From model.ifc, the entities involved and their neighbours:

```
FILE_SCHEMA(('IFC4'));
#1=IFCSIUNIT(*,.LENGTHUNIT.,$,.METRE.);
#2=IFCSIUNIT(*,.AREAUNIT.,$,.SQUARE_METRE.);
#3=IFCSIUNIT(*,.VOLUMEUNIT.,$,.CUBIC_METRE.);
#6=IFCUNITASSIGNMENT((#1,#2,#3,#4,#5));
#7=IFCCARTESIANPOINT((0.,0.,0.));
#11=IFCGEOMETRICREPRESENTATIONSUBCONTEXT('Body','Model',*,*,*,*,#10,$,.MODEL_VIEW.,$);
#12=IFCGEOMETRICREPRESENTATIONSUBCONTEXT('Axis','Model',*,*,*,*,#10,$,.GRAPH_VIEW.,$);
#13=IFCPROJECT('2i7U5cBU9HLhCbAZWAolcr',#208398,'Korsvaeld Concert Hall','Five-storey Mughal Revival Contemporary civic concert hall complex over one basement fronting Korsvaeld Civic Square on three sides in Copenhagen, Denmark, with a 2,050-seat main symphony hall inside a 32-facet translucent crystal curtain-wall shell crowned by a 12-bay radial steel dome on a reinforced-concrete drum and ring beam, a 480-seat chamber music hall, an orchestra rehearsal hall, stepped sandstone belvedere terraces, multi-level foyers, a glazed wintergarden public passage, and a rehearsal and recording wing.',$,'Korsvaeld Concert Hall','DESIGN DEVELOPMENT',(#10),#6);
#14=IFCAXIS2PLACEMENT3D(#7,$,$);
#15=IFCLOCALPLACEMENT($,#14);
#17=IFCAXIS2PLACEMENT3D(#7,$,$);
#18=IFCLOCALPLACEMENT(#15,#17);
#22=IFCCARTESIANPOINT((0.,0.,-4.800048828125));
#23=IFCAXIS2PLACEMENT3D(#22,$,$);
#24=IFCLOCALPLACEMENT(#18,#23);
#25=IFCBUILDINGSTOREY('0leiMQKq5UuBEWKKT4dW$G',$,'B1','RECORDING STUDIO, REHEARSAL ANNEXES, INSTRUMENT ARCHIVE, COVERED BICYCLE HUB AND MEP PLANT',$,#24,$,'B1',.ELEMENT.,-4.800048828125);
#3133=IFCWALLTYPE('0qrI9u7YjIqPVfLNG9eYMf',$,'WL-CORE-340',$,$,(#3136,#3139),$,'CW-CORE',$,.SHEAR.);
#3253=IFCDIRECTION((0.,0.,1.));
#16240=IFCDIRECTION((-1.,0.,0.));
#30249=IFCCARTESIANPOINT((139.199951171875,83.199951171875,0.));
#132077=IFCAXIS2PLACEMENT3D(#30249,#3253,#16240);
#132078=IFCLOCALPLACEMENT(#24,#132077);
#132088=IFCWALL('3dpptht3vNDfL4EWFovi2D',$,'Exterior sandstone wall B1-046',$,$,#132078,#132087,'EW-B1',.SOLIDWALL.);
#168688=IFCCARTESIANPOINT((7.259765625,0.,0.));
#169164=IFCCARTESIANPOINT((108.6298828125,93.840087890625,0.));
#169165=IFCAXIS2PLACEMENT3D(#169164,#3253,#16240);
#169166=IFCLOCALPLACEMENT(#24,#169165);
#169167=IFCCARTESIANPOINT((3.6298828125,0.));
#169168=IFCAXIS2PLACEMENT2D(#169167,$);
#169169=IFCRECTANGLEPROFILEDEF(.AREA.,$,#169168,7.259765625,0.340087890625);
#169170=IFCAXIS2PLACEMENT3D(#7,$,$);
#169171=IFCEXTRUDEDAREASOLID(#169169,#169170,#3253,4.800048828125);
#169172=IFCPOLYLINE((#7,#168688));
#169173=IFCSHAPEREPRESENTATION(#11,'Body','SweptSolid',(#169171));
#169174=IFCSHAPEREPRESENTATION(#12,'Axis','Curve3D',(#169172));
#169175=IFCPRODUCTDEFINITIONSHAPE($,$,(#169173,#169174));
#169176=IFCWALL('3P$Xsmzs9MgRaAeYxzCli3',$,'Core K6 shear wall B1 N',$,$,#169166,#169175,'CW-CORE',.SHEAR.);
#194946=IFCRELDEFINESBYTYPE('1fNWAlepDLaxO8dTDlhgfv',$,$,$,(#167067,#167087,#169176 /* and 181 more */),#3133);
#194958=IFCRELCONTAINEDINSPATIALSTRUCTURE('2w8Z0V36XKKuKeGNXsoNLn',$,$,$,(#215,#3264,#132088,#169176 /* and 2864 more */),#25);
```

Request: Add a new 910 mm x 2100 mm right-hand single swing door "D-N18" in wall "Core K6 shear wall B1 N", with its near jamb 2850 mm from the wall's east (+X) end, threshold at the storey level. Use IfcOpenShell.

```python
import numpy as np
import ifcopenshell
import ifcopenshell.api.feature
import ifcopenshell.api.geometry
import ifcopenshell.api.root
import ifcopenshell.api.spatial
import ifcopenshell.geom
import ifcopenshell.util.element
import ifcopenshell.util.placement
import ifcopenshell.util.representation
import ifcopenshell.util.shape
import ifcopenshell.util.unit

model = ifcopenshell.open("model.ifc")
unit_scale = ifcopenshell.util.unit.calculate_unit_scale(model)
settings = ifcopenshell.geom.settings()


def volume(element):
    """Net volume in cubic metres, openings subtracted."""
    shape = ifcopenshell.geom.create_shape(settings, element)
    return ifcopenshell.util.shape.get_volume(shape.geometry)


wall = model.by_guid("3P$Xsmzs9MgRaAeYxzCli3")
storey = ifcopenshell.util.element.get_container(wall, ifc_class="IfcBuildingStorey")
context = ifcopenshell.util.representation.get_context(model, "Model", "Body", "MODEL_VIEW")
before = volume(wall)

width, height, from_end, sill = 0.91, 2.1, 2.85, 0.0  # metres

# The wall runs along its own X axis, and the end named is its -X end.
wall_shape = ifcopenshell.geom.create_shape(settings, wall)
x, y, z = ifcopenshell.util.shape.get_vertices(wall_shape.geometry).T
start = x.min() + from_end
face, thickness = float(y.min()), float(y.max() - y.min())
wall_matrix = ifcopenshell.util.placement.get_local_placement(wall.ObjectPlacement)
level = ifcopenshell.util.placement.get_local_placement(storey.ObjectPlacement)[2, 3]


def in_wall(x, y):
    """Placement at x, y metres in the wall's axes, at sill height."""
    matrix = wall_matrix.copy()
    matrix[:, 3] = wall_matrix @ np.array([x / unit_scale, y / unit_scale, 0.0, 1.0])
    matrix[2, 3] = level + sill / unit_scale
    return matrix


# Opening: a box that overshoots both wall faces by 50 mm.
opening = ifcopenshell.api.root.create_entity(model, ifc_class="IfcOpeningElement", predefined_type="OPENING")
box = ifcopenshell.api.geometry.add_wall_representation(
    model, context=context, length=width, height=height, thickness=thickness + 0.1
)
ifcopenshell.api.geometry.assign_representation(model, product=opening, representation=box)
ifcopenshell.api.geometry.edit_object_placement(model, product=opening, matrix=in_wall(start, face - 0.05), is_si=False)
ifcopenshell.api.feature.add_feature(model, feature=opening, element=wall)

door = ifcopenshell.api.root.create_entity(model, ifc_class="IfcDoor", name="D-N18", predefined_type="DOOR")
door.OverallWidth, door.OverallHeight = width / unit_scale, height / unit_scale
door.OperationType = "SINGLE_SWING_RIGHT"
body = ifcopenshell.api.geometry.add_door_representation(
    model,
    context=context,
    overall_width=door.OverallWidth,
    overall_height=door.OverallHeight,
    operation_type="SINGLE_SWING_RIGHT",
    lining_properties={"LiningDepth": thickness / unit_scale, "ThresholdDepth": thickness / unit_scale},
)
ifcopenshell.api.geometry.assign_representation(model, product=door, representation=body)
ifcopenshell.api.spatial.assign_container(model, products=[door], relating_structure=storey)
ifcopenshell.api.feature.add_filling(model, opening=opening, element=door)

# The lining spans the wall, so the door starts at the wall face.
ifcopenshell.api.geometry.edit_object_placement(model, product=door, matrix=in_wall(start, face), is_si=False)

after = volume(wall)

print(f"wall volume {before:.3f} -> {after:.3f} m3")

model.write("model_edited.ifc")
```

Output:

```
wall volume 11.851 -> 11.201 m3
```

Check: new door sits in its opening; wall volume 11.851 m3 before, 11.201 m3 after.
